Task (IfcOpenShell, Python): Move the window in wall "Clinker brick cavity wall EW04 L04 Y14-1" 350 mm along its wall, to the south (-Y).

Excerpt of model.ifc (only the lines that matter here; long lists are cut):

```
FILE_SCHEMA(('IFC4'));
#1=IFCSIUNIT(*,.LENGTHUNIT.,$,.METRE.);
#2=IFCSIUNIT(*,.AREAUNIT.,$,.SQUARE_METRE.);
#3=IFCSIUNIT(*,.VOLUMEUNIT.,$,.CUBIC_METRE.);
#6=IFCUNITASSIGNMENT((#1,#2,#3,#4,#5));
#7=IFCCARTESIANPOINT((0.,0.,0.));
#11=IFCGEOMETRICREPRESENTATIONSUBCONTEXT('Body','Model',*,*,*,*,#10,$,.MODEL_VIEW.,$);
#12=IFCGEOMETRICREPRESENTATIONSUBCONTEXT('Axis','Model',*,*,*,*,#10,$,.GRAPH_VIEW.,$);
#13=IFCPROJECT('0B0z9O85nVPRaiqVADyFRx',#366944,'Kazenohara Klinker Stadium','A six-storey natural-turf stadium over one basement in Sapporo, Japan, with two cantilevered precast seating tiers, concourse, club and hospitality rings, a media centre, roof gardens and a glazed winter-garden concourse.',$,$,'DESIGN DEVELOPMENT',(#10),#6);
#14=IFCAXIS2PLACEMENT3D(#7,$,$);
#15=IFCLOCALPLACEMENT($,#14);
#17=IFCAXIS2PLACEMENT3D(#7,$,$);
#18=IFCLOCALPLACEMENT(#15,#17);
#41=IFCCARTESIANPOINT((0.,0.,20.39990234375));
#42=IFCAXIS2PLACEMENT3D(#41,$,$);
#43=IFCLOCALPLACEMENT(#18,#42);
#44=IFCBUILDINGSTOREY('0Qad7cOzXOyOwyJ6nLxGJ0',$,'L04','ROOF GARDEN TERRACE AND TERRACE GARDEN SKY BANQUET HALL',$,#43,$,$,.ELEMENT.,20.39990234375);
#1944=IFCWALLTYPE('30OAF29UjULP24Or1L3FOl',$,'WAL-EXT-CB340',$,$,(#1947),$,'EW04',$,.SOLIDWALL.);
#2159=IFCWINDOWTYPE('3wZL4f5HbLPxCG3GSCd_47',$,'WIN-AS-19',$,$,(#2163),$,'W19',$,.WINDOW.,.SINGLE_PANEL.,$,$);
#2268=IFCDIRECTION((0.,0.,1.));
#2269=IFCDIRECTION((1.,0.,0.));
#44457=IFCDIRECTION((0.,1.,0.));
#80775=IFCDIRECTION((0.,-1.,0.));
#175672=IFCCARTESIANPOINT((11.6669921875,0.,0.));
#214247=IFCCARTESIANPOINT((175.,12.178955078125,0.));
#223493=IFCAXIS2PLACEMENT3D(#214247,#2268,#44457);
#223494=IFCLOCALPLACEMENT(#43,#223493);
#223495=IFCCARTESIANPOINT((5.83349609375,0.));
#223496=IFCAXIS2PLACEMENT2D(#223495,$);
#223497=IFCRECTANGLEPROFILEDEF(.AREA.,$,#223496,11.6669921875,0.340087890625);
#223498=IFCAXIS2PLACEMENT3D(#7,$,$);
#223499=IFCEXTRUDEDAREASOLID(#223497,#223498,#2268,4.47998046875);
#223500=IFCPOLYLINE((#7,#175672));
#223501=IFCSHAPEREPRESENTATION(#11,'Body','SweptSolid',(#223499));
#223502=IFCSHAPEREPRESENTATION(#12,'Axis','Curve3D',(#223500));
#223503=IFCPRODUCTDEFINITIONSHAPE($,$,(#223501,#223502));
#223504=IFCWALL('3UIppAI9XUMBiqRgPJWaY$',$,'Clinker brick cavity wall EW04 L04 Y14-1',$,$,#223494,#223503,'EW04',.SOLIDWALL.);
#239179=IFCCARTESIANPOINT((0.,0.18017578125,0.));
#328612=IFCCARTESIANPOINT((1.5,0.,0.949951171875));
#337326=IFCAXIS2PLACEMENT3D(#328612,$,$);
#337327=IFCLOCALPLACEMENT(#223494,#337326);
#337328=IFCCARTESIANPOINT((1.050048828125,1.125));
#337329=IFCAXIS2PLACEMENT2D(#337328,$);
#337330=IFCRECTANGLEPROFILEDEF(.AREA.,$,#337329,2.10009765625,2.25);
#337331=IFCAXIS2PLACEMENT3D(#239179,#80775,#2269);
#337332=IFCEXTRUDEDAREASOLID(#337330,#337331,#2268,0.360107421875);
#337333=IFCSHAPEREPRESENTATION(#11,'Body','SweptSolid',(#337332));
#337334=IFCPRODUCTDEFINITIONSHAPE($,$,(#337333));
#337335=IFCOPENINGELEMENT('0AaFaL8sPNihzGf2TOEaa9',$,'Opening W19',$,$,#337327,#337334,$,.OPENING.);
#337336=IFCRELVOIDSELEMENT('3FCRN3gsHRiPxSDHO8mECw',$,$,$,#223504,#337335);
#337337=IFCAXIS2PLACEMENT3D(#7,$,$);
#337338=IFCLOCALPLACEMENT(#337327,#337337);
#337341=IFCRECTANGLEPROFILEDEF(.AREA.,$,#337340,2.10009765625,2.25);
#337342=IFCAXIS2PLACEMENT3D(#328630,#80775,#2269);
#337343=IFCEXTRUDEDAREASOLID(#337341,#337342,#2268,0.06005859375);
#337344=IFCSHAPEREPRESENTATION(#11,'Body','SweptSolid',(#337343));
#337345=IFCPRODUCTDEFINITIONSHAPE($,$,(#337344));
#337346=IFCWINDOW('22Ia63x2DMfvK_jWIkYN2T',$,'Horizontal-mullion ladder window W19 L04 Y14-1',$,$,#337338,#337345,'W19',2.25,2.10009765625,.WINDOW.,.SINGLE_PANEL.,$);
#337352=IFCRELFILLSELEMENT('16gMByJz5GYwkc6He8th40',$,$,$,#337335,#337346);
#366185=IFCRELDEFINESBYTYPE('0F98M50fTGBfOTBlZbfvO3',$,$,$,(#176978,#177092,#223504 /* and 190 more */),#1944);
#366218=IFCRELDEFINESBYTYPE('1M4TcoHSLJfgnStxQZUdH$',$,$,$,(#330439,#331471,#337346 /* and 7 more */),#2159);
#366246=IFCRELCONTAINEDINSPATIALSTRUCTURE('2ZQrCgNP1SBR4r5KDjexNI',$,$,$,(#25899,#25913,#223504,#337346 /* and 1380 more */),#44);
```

```python
import ifcopenshell
import ifcopenshell.api.geometry
import ifcopenshell.util.placement
import ifcopenshell.util.unit

model = ifcopenshell.open("model.ifc")
unit_scale = ifcopenshell.util.unit.calculate_unit_scale(model)

window = model.by_guid("22Ia63x2DMfvK_jWIkYN2T")
opening = window.FillsVoids[0].RelatingOpeningElement
wall = opening.VoidsElements[0].RelatingBuildingElement

wall_matrix = ifcopenshell.util.placement.get_local_placement(wall.ObjectPlacement)
shift = wall_matrix[:3, 0] * -0.35 / unit_scale
before = ifcopenshell.util.placement.get_local_placement(window.ObjectPlacement)[:3, 3].copy()

# The window is placed relative to its opening, so it follows when the opening moves.
matrix = ifcopenshell.util.placement.get_local_placement(opening.ObjectPlacement)
matrix[:3, 3] += shift
ifcopenshell.api.geometry.edit_object_placement(
    model, product=opening, matrix=matrix, is_si=False, should_transform_children=True
)

after = ifcopenshell.util.placement.get_local_placement(window.ObjectPlacement)[:3, 3]
print("window moved by", (after - before).round(3) + 0.0)

model.write("model-out.ifc")
```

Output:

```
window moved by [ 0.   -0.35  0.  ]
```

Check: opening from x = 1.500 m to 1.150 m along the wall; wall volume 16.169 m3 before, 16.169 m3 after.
